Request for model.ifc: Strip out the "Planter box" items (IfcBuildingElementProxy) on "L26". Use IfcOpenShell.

First a look at what the model holds.

```python
import ifcopenshell
import ifcopenshell.util.element

model = ifcopenshell.open("model.ifc")
print(model.schema)
storey = next(s for s in model.by_type("IfcBuildingStorey") if s.Name == "L26")
proxies = [e for e in ifcopenshell.util.element.get_decomposition(storey) if e.is_a("IfcBuildingElementProxy")]
seen = {}
for e in proxies:
    element_type = ifcopenshell.util.element.get_type(e)
    name = element_type.Name if element_type not in (None, e) else None
    seen[name] = seen.get(name, 0) + 1
for name, count in sorted(seen.items(), key=str):
    print(count, "x", name)
```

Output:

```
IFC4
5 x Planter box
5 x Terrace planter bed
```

```python
import ifcopenshell
import ifcopenshell.api.root
import ifcopenshell.util.element

model = ifcopenshell.open("model.ifc")

storey = next(s for s in model.by_type("IfcBuildingStorey") if s.Name == "L26")
proxies = [e for e in ifcopenshell.util.element.get_decomposition(storey) if e.is_a("IfcBuildingElementProxy")]
targets = [e for e in proxies if (t := ifcopenshell.util.element.get_type(e)) not in (None, e) and t.Name == "Planter box"]

for e in targets:
    ifcopenshell.api.root.remove_product(model, product=e)
print(len(targets), "removed")

model.write("model-out.ifc")
```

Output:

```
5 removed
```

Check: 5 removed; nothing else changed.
